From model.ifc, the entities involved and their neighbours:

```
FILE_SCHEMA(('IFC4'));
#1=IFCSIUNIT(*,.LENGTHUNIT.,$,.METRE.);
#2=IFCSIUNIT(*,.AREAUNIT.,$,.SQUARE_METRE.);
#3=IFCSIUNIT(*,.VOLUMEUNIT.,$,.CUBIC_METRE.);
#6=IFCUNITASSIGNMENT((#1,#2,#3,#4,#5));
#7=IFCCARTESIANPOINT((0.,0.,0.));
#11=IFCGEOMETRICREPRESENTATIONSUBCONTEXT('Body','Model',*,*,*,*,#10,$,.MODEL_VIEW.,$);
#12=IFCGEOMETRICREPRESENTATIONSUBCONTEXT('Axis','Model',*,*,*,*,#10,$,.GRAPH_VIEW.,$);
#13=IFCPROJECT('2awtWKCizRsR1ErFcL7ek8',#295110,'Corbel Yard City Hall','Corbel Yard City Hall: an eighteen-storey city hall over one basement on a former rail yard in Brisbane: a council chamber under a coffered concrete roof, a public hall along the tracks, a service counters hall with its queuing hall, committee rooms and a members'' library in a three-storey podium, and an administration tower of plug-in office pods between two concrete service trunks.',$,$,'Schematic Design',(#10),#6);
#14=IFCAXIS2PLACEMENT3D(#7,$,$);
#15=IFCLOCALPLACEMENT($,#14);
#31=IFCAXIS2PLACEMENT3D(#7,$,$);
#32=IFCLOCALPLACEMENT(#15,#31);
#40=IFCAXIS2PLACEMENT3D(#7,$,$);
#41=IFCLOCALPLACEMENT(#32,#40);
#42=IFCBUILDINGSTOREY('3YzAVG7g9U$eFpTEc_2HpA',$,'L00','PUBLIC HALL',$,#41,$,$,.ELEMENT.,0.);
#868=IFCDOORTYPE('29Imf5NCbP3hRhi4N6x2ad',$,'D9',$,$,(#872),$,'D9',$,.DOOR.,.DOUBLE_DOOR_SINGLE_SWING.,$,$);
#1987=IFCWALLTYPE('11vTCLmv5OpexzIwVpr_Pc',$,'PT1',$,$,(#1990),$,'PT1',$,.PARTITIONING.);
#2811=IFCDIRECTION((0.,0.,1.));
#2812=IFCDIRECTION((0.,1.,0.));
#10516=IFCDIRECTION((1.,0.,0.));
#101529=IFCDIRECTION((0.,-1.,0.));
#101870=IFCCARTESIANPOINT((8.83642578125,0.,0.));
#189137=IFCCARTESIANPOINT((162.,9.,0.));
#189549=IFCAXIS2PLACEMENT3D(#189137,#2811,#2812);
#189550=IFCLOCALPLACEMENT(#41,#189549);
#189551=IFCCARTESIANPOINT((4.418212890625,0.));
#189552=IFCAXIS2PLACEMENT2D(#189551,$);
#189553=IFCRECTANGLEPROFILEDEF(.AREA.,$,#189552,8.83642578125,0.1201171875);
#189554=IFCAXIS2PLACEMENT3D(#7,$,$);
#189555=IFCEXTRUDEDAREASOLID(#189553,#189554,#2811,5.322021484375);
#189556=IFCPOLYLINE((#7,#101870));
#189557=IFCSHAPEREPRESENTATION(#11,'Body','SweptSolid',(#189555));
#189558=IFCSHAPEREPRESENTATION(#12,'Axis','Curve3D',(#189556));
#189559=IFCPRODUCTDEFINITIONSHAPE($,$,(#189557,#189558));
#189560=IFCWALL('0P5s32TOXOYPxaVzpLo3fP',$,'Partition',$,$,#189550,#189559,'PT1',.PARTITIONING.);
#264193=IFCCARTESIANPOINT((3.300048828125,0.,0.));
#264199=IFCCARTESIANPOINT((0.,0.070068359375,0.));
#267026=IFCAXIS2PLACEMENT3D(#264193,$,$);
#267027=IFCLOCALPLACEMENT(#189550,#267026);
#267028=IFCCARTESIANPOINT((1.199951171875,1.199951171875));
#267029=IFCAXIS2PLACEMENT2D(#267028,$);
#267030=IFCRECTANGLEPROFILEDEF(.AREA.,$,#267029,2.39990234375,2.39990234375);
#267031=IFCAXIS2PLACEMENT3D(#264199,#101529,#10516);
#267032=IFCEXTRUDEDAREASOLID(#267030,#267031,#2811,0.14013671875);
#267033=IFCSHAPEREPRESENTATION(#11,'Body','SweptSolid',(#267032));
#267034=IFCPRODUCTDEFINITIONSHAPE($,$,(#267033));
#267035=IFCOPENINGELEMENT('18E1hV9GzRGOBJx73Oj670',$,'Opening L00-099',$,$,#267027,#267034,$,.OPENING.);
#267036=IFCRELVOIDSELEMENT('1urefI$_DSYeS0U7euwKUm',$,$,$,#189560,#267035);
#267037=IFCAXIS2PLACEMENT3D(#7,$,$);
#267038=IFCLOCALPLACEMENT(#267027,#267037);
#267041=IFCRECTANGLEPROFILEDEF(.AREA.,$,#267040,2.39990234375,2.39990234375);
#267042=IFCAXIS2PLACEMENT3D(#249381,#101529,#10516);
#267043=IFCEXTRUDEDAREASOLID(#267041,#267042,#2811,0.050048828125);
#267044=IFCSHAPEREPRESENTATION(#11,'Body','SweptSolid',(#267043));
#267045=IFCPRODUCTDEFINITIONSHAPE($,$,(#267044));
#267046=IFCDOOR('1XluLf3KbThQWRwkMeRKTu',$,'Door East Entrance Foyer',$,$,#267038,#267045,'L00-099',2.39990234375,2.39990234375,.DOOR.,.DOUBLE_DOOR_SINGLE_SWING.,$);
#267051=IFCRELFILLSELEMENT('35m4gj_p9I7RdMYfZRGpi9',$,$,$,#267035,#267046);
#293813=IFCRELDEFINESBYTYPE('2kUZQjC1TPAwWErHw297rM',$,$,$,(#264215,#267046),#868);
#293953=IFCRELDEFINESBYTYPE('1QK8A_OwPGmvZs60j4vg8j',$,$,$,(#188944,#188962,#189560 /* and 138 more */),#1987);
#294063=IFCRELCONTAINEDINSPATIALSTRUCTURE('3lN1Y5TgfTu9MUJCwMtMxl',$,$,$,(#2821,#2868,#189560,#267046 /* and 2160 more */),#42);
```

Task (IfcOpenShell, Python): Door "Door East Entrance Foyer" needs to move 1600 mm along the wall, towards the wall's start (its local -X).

```python
import ifcopenshell
import ifcopenshell.api.geometry
import ifcopenshell.util.placement
import ifcopenshell.util.unit

model = ifcopenshell.open("model.ifc")
unit_scale = ifcopenshell.util.unit.calculate_unit_scale(model)

door = model.by_guid("1XluLf3KbThQWRwkMeRKTu")
opening = door.FillsVoids[0].RelatingOpeningElement
wall = opening.VoidsElements[0].RelatingBuildingElement

wall_matrix = ifcopenshell.util.placement.get_local_placement(wall.ObjectPlacement)
shift = wall_matrix[:3, 0] * -1.6 / unit_scale
before = ifcopenshell.util.placement.get_local_placement(door.ObjectPlacement)[:3, 3].copy()

# The door is placed relative to its opening, so it follows when the opening moves.
matrix = ifcopenshell.util.placement.get_local_placement(opening.ObjectPlacement)
matrix[:3, 3] += shift
ifcopenshell.api.geometry.edit_object_placement(
    model, product=opening, matrix=matrix, is_si=False, should_transform_children=True
)

after = ifcopenshell.util.placement.get_local_placement(door.ObjectPlacement)[:3, 3]
print("door moved by", (after - before).round(3) + 0.0)

model.write("model-out.ifc")
```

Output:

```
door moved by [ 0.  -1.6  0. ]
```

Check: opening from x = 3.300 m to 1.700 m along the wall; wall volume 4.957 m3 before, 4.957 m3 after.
